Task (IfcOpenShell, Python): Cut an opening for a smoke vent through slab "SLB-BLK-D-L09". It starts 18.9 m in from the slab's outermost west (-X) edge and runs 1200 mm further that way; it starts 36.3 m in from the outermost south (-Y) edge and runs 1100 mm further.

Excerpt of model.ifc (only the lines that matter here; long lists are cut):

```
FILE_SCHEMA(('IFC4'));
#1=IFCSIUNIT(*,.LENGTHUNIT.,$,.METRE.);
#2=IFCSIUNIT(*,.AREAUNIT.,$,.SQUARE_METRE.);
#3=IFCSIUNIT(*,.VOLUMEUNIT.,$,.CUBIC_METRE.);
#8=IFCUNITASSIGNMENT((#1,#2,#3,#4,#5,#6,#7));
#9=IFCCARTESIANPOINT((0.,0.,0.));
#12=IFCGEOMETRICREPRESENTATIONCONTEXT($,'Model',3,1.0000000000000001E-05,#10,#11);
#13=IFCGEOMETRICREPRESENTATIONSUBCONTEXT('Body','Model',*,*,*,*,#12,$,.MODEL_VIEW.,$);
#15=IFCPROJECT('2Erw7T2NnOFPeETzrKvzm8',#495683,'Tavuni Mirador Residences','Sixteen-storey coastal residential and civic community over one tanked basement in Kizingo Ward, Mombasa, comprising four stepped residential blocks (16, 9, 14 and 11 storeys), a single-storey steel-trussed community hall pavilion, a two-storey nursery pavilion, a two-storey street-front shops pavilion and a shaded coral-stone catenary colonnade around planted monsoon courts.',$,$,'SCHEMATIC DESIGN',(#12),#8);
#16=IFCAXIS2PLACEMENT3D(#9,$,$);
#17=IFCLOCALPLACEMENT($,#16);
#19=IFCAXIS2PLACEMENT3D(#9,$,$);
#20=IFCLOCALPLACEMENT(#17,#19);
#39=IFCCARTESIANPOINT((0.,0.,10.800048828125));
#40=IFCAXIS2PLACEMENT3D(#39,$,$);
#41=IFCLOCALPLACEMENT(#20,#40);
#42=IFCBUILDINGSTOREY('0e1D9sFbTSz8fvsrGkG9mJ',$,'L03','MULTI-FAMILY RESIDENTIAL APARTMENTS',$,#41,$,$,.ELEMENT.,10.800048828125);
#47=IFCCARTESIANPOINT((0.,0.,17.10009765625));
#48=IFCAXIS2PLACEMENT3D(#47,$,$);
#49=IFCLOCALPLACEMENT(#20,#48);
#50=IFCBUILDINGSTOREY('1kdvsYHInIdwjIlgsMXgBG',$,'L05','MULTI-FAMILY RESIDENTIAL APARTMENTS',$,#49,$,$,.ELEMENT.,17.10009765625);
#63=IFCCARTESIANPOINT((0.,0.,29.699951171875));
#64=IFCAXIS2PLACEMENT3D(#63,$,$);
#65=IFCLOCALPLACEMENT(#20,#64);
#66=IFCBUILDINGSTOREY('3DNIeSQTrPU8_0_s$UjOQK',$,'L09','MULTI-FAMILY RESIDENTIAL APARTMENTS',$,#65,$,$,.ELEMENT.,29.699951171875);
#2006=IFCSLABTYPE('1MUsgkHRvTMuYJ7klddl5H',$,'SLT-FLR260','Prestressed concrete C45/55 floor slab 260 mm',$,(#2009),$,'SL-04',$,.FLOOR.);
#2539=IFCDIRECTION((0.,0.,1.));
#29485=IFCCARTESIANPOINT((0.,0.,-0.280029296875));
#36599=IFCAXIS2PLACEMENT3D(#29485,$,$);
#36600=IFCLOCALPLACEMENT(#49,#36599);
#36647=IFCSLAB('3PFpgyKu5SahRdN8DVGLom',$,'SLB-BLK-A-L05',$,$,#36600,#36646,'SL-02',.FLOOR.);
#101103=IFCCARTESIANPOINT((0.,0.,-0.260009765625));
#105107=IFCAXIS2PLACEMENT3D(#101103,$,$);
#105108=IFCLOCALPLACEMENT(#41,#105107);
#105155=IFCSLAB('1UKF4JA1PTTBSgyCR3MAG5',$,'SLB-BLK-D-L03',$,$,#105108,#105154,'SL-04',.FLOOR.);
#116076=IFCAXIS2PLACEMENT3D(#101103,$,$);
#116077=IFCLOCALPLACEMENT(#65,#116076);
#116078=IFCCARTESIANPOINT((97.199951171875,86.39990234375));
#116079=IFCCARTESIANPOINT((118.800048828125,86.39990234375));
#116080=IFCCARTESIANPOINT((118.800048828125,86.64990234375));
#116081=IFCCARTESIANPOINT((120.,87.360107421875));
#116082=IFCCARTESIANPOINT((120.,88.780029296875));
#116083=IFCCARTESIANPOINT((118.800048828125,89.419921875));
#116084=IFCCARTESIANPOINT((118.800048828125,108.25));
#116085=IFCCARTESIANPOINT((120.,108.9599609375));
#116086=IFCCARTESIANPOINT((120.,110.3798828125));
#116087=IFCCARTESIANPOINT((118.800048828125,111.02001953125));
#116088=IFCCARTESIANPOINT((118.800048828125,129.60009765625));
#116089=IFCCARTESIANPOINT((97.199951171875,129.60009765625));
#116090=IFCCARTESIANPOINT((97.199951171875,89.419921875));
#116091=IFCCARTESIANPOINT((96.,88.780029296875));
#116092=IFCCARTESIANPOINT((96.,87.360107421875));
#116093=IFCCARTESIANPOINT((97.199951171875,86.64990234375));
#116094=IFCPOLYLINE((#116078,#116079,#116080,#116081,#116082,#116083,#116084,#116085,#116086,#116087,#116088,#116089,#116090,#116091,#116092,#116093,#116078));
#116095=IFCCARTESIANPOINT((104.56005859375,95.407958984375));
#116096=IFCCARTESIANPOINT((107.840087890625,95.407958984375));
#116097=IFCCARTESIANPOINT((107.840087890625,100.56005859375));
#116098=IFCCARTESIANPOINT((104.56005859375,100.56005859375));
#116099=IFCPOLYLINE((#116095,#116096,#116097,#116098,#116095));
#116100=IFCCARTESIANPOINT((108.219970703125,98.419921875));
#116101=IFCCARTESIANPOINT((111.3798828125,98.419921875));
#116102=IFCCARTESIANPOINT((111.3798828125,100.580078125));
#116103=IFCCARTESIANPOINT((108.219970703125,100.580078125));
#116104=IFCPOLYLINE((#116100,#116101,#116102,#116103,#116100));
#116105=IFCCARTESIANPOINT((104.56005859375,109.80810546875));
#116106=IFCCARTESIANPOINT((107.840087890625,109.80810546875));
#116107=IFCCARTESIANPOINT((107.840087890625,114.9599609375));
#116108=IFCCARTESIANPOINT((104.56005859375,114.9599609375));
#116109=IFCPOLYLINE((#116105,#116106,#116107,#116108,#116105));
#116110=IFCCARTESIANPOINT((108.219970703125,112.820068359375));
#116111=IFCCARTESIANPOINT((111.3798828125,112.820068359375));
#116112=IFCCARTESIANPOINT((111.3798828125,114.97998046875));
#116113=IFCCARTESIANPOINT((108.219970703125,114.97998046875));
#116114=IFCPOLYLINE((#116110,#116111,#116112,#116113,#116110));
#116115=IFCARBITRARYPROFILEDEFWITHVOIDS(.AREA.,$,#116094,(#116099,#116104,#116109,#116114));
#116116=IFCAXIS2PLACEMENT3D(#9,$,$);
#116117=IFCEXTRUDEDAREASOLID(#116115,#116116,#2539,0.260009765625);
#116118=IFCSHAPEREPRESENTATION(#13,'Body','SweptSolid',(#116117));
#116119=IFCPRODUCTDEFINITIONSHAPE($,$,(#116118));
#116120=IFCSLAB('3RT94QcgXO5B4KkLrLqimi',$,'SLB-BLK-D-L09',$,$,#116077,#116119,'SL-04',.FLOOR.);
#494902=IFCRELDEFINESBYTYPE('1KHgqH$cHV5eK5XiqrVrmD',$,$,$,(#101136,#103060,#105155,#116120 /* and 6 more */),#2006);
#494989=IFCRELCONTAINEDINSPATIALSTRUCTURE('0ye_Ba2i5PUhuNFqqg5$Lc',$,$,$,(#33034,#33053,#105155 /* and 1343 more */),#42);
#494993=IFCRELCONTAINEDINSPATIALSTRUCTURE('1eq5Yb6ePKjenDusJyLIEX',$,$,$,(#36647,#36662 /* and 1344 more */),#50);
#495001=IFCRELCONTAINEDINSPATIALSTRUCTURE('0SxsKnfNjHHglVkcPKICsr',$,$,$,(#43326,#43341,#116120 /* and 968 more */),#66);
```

```python
import numpy as np
import ifcopenshell
import ifcopenshell.api.feature
import ifcopenshell.api.geometry
import ifcopenshell.api.root
import ifcopenshell.geom
import ifcopenshell.util.placement
import ifcopenshell.util.representation
import ifcopenshell.util.shape
import ifcopenshell.util.unit

model = ifcopenshell.open("model.ifc")
unit_scale = ifcopenshell.util.unit.calculate_unit_scale(model)
settings = ifcopenshell.geom.settings()


def volume(element):
    """Net volume in cubic metres, openings subtracted."""
    shape = ifcopenshell.geom.create_shape(settings, element)
    return ifcopenshell.util.shape.get_volume(shape.geometry)


slab = model.by_guid("3RT94QcgXO5B4KkLrLqimi")
before = volume(slab)

# Extent in the slab's own axes, in metres. The edges named are its -X and -Y sides.
slab_shape = ifcopenshell.geom.create_shape(settings, slab)
vertices = ifcopenshell.util.shape.get_vertices(slab_shape.geometry)
x_min, y_min, bottom = vertices.min(axis=0)
top = vertices[:, 2].max()

opening = ifcopenshell.api.root.create_entity(model, ifc_class="IfcOpeningElement", name="Smoke vent opening", predefined_type="OPENING")
context = ifcopenshell.util.representation.get_context(model, "Model", "Body", "MODEL_VIEW")
width, depth = 1.2, 1.1
outline = [(0.0, 0.0), (width, 0.0), (width, depth), (0.0, depth), (0.0, 0.0)]
# Overshoot both faces by 50 mm so the cut is clean.
shape = ifcopenshell.api.geometry.add_slab_representation(
    model, context=context, depth=top - bottom + 0.1, polyline=outline
)
ifcopenshell.api.geometry.assign_representation(model, product=opening, representation=shape)

matrix = ifcopenshell.util.placement.get_local_placement(slab.ObjectPlacement)
matrix[:, 3] = matrix @ np.append(np.array([x_min + 18.9, y_min + 36.3, bottom - 0.05]) / unit_scale, 1.0)
ifcopenshell.api.geometry.edit_object_placement(model, product=opening, matrix=matrix, is_si=False)
ifcopenshell.api.feature.add_feature(model, feature=opening, element=slab)

after = volume(slab)

print(f"slab volume {before:.3f} -> {after:.3f} m3")

model.write("model_rev.ifc")
```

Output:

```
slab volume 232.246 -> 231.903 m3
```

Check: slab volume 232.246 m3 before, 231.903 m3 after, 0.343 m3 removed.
